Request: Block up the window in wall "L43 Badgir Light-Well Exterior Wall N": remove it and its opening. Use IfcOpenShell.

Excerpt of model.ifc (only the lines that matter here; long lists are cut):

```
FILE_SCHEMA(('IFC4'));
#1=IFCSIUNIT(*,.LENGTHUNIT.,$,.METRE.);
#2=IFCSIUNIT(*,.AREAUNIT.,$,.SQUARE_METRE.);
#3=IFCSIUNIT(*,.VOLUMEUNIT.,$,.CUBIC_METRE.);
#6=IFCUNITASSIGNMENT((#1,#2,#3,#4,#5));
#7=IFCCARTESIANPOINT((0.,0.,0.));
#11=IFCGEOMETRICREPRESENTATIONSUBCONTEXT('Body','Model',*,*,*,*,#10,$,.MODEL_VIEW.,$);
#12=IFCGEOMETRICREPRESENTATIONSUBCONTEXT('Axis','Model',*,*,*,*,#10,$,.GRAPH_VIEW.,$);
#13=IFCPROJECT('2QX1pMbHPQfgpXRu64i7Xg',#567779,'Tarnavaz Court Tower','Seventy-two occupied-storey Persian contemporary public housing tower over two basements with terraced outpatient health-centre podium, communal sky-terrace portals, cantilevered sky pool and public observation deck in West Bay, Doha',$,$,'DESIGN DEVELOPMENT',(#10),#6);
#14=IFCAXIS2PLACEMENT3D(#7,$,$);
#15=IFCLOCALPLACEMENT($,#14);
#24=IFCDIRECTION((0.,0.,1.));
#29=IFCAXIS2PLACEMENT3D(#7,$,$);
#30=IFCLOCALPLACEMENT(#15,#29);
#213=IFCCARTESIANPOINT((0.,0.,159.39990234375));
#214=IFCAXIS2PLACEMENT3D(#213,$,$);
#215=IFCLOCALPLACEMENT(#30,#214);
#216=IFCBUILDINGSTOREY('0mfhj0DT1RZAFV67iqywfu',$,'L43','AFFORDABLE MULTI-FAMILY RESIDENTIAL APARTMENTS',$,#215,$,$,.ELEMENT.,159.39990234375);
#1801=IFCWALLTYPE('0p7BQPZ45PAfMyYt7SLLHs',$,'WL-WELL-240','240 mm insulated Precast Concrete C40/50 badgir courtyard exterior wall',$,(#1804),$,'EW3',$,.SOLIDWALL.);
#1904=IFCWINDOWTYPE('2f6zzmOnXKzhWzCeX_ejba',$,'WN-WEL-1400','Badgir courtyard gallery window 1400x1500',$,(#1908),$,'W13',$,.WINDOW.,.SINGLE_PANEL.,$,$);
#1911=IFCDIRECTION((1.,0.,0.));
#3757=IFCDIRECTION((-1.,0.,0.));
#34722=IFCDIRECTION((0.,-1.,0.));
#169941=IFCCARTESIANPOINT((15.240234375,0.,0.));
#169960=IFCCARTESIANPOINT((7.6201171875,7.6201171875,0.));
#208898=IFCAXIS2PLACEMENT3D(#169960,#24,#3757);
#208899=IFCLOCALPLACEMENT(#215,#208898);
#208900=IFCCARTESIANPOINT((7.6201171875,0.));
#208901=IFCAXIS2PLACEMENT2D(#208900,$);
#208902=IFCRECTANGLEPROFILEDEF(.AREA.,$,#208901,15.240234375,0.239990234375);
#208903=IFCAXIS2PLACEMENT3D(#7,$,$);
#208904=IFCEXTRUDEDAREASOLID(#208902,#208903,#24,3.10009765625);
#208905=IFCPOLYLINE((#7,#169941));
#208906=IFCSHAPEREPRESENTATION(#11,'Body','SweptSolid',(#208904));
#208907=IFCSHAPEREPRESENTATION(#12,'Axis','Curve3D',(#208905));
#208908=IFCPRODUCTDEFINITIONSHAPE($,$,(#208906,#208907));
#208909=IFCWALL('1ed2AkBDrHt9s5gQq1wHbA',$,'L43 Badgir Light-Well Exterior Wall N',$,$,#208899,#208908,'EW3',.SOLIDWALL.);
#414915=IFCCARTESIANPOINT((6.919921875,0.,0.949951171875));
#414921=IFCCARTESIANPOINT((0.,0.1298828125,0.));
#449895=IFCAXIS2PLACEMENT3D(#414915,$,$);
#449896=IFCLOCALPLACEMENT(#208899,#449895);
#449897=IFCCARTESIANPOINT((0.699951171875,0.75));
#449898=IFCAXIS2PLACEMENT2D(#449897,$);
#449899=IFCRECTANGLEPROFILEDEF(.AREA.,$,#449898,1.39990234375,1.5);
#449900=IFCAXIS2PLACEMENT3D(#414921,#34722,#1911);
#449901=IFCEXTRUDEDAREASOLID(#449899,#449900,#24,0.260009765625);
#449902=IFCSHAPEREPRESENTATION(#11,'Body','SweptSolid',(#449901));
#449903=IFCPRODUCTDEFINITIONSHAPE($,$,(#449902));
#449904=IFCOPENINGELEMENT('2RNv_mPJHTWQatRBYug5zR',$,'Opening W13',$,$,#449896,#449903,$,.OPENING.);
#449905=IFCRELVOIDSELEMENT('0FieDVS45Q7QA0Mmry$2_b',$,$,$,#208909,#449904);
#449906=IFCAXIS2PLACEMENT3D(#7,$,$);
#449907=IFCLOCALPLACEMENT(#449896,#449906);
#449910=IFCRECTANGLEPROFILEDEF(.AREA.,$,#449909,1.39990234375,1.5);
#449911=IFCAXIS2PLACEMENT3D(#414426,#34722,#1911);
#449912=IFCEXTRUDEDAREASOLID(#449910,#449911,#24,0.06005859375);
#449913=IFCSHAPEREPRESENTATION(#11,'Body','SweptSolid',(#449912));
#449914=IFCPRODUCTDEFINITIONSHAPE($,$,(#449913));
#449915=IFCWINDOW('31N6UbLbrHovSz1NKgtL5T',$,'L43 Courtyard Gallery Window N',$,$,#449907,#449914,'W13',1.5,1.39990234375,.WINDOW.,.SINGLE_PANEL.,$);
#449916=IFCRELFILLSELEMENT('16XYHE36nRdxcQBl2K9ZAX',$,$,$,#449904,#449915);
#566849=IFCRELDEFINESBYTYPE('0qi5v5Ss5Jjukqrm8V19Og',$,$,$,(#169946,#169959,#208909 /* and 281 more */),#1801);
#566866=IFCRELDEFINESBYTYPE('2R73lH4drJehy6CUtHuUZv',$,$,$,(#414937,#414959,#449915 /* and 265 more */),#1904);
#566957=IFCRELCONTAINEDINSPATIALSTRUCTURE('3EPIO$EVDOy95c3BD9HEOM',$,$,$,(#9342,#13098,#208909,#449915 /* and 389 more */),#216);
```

```python
import ifcopenshell
import ifcopenshell.api.feature
import ifcopenshell.api.root
import ifcopenshell.geom
import ifcopenshell.util.shape

model = ifcopenshell.open("model.ifc")
settings = ifcopenshell.geom.settings()


def volume(element):
    """Net volume in cubic metres, openings subtracted."""
    shape = ifcopenshell.geom.create_shape(settings, element)
    return ifcopenshell.util.shape.get_volume(shape.geometry)


window = model.by_guid("31N6UbLbrHovSz1NKgtL5T")
opening = window.FillsVoids[0].RelatingOpeningElement
wall = opening.VoidsElements[0].RelatingBuildingElement
before = volume(wall)

ifcopenshell.api.root.remove_product(model, product=window)
ifcopenshell.api.feature.remove_feature(model, feature=opening)

after = volume(wall)

print(f"wall volume {before:.3f} -> {after:.3f} m3")

model.write("model_v2.ifc")
```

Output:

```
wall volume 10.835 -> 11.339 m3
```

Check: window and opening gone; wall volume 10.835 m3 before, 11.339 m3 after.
